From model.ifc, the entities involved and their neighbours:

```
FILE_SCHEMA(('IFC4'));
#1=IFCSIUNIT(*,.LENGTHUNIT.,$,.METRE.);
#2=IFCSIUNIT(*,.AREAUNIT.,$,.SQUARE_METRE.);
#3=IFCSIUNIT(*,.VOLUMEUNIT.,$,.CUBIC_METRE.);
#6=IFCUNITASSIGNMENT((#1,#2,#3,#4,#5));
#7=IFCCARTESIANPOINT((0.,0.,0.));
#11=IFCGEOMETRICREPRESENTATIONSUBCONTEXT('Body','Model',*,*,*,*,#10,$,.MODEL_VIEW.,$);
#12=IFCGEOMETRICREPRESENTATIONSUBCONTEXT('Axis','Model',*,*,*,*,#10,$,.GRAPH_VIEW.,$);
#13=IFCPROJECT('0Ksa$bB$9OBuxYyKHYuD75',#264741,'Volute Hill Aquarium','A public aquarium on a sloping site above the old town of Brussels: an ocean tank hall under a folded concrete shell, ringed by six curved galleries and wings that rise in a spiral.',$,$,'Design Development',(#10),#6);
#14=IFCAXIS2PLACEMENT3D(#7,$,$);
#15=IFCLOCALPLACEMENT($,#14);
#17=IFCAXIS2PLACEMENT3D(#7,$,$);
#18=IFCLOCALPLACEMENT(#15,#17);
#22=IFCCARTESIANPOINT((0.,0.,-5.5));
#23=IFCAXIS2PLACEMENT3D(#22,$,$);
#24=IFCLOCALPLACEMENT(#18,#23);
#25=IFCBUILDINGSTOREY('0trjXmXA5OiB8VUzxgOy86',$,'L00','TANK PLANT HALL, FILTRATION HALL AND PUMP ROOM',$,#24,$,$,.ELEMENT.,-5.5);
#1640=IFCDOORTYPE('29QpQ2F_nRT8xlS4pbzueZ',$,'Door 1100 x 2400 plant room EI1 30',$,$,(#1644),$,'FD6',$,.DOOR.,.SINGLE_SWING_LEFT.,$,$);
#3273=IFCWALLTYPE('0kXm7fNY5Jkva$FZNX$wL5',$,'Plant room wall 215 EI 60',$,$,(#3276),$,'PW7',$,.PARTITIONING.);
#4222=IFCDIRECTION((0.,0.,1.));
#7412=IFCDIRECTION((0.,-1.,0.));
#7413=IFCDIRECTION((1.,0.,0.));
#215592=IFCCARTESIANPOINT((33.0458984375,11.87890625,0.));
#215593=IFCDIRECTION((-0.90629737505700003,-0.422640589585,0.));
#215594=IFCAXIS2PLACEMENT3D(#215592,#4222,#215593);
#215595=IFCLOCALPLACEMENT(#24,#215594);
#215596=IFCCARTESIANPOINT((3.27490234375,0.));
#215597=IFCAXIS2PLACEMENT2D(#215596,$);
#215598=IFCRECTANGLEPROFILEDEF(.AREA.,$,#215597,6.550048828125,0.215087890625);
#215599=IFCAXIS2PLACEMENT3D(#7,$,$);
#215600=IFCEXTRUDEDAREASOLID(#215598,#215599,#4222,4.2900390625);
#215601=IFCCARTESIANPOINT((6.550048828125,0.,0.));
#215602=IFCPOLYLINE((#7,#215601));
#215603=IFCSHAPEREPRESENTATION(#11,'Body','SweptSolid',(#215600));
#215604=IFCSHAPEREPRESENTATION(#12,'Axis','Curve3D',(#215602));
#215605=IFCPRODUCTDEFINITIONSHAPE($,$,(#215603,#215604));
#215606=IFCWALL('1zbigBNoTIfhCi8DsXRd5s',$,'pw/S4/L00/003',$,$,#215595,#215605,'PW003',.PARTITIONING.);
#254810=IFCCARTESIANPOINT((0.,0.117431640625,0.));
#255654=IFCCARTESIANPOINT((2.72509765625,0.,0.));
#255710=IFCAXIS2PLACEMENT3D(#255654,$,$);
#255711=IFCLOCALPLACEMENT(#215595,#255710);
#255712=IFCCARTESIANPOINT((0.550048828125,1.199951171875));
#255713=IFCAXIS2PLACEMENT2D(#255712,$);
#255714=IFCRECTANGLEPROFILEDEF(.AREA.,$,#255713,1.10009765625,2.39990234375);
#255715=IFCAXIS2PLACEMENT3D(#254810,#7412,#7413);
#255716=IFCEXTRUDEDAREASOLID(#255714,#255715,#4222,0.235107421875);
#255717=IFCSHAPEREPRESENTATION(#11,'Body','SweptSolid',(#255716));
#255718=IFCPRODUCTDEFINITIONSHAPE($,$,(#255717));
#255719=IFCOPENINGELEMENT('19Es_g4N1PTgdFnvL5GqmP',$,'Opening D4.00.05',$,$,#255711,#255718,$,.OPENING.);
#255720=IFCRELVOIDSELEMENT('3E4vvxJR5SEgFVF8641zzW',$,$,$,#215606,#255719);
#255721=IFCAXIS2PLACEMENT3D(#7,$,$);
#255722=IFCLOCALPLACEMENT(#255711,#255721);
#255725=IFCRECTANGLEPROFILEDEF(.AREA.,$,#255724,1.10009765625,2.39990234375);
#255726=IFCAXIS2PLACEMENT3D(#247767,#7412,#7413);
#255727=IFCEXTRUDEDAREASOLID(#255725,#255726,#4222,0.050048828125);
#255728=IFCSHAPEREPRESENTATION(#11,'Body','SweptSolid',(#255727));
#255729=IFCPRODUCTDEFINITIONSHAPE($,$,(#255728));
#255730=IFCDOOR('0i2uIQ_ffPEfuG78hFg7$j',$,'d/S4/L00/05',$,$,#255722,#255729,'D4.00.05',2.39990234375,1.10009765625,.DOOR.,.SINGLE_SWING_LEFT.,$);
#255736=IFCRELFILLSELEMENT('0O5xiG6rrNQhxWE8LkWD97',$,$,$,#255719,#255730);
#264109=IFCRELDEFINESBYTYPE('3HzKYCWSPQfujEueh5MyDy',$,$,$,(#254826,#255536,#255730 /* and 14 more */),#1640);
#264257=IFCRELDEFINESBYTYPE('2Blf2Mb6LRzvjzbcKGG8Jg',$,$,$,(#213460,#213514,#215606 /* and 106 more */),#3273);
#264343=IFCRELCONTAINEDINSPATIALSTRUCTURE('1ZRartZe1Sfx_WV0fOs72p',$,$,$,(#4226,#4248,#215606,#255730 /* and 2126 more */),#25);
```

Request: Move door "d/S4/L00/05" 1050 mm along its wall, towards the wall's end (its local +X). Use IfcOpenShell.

```python
import ifcopenshell
import ifcopenshell.api.geometry
import ifcopenshell.util.placement
import ifcopenshell.util.unit

model = ifcopenshell.open("model.ifc")
unit_scale = ifcopenshell.util.unit.calculate_unit_scale(model)

door = model.by_guid("0i2uIQ_ffPEfuG78hFg7$j")
opening = door.FillsVoids[0].RelatingOpeningElement
wall = opening.VoidsElements[0].RelatingBuildingElement

wall_matrix = ifcopenshell.util.placement.get_local_placement(wall.ObjectPlacement)
shift = wall_matrix[:3, 0] * 1.05 / unit_scale
before = ifcopenshell.util.placement.get_local_placement(door.ObjectPlacement)[:3, 3].copy()

# The door is placed relative to its opening, so it follows when the opening moves.
matrix = ifcopenshell.util.placement.get_local_placement(opening.ObjectPlacement)
matrix[:3, 3] += shift
ifcopenshell.api.geometry.edit_object_placement(
    model, product=opening, matrix=matrix, is_si=False, should_transform_children=True
)

after = ifcopenshell.util.placement.get_local_placement(door.ObjectPlacement)[:3, 3]
print("door moved by", (after - before).round(3) + 0.0)

model.write("model-out.ifc")
```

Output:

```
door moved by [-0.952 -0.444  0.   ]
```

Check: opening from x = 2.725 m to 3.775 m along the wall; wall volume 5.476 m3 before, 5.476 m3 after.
